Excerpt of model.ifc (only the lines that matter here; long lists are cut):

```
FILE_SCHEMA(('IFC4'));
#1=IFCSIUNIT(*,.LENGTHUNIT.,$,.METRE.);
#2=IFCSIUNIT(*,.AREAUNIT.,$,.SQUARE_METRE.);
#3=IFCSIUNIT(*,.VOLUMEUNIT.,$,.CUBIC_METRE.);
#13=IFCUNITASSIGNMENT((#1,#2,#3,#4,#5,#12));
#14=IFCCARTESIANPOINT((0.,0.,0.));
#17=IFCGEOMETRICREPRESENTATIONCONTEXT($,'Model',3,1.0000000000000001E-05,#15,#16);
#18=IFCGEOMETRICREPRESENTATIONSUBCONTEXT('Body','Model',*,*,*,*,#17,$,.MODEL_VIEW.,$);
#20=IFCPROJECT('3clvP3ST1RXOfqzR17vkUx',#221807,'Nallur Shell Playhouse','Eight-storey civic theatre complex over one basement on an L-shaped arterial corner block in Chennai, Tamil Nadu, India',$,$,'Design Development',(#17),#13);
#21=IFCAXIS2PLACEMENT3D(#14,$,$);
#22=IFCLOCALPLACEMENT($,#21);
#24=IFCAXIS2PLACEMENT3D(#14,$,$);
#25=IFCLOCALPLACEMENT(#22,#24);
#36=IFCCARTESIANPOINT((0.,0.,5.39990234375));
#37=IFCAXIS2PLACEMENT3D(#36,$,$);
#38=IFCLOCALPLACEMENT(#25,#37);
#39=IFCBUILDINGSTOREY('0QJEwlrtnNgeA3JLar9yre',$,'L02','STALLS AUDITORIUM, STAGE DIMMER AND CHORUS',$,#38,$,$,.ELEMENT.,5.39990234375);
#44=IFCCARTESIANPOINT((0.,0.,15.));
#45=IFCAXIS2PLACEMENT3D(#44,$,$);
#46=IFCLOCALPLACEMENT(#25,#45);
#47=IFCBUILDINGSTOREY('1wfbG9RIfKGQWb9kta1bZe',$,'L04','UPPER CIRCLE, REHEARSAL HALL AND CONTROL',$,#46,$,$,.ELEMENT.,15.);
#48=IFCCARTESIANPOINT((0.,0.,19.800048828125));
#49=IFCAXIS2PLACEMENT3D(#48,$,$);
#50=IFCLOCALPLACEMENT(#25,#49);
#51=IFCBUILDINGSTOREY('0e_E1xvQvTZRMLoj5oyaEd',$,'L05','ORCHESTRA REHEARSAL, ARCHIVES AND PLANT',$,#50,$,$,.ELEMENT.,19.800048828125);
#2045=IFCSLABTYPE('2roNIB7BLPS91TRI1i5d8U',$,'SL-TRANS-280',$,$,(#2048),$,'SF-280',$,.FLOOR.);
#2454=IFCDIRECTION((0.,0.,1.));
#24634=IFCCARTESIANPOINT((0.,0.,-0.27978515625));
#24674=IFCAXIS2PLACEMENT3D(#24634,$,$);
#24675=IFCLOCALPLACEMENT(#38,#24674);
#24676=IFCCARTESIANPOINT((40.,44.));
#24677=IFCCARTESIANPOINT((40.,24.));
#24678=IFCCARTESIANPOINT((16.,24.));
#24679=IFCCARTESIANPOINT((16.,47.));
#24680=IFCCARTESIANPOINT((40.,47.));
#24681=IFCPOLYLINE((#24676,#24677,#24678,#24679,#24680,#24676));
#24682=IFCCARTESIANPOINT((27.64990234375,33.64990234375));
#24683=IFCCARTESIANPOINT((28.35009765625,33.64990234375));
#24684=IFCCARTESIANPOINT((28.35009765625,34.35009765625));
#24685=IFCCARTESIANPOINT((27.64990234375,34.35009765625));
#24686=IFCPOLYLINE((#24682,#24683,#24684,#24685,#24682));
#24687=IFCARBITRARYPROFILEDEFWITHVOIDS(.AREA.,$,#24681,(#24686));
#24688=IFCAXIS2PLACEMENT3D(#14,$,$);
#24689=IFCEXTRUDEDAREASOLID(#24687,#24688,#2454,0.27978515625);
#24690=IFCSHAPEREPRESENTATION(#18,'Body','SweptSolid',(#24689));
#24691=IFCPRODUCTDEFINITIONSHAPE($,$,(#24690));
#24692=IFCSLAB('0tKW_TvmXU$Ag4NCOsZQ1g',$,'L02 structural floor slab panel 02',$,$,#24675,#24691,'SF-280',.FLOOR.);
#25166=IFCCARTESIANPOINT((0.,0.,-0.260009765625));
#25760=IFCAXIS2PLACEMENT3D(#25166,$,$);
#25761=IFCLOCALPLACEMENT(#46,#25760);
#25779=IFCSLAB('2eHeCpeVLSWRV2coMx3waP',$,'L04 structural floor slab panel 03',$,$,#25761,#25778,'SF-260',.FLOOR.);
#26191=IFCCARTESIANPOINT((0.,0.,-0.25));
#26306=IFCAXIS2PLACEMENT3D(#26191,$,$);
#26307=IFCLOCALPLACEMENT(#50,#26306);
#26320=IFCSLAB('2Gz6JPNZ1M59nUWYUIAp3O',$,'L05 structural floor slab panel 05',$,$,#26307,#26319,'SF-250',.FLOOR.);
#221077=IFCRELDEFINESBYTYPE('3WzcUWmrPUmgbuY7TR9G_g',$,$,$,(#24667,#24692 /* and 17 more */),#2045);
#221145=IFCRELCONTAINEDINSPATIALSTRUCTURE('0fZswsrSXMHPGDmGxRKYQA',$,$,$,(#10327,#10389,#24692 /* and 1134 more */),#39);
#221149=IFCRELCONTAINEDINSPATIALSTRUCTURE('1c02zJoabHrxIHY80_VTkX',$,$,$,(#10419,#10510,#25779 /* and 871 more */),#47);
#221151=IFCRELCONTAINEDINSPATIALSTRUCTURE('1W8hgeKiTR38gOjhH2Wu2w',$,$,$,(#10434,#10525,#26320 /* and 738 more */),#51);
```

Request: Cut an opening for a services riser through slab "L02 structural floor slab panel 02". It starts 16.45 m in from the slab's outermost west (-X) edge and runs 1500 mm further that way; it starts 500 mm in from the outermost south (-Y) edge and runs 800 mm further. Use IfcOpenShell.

```python
import numpy as np
import ifcopenshell
import ifcopenshell.api.feature
import ifcopenshell.api.geometry
import ifcopenshell.api.root
import ifcopenshell.geom
import ifcopenshell.util.placement
import ifcopenshell.util.representation
import ifcopenshell.util.shape
import ifcopenshell.util.unit

model = ifcopenshell.open("model.ifc")
unit_scale = ifcopenshell.util.unit.calculate_unit_scale(model)
settings = ifcopenshell.geom.settings()


def volume(element):
    """Net volume in cubic metres, openings subtracted."""
    shape = ifcopenshell.geom.create_shape(settings, element)
    return ifcopenshell.util.shape.get_volume(shape.geometry)


slab = model.by_guid("0tKW_TvmXU$Ag4NCOsZQ1g")
before = volume(slab)

# Extent in the slab's own axes, in metres. The edges named are its -X and -Y sides.
slab_shape = ifcopenshell.geom.create_shape(settings, slab)
vertices = ifcopenshell.util.shape.get_vertices(slab_shape.geometry)
x_min, y_min, bottom = vertices.min(axis=0)
top = vertices[:, 2].max()

opening = ifcopenshell.api.root.create_entity(model, ifc_class="IfcOpeningElement", name="Services riser opening", predefined_type="OPENING")
context = ifcopenshell.util.representation.get_context(model, "Model", "Body", "MODEL_VIEW")
width, depth = 1.5, 0.8
outline = [(0.0, 0.0), (width, 0.0), (width, depth), (0.0, depth), (0.0, 0.0)]
# Overshoot both faces by 50 mm so the cut is clean.
shape = ifcopenshell.api.geometry.add_slab_representation(
    model, context=context, depth=top - bottom + 0.1, polyline=outline
)
ifcopenshell.api.geometry.assign_representation(model, product=opening, representation=shape)

matrix = ifcopenshell.util.placement.get_local_placement(slab.ObjectPlacement)
matrix[:, 3] = matrix @ np.append(np.array([x_min + 16.45, y_min + 0.5, bottom - 0.05]) / unit_scale, 1.0)
ifcopenshell.api.geometry.edit_object_placement(model, product=opening, matrix=matrix, is_si=False)
ifcopenshell.api.feature.add_feature(model, feature=opening, element=slab)

after = volume(slab)

print(f"slab volume {before:.3f} -> {after:.3f} m3")

model.write("model_edited.ifc")
```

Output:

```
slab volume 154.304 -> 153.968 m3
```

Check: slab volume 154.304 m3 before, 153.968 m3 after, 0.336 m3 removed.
